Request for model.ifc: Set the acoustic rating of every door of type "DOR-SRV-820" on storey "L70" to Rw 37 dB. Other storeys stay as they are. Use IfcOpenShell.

First a look at what the model holds.

```python
import ifcopenshell
import ifcopenshell.util.element

model = ifcopenshell.open("model.ifc")
print(model.schema)
storey = next(s for s in model.by_type("IfcBuildingStorey") if s.Name == "L70")
doors = [e for e in ifcopenshell.util.element.get_decomposition(storey) if e.is_a("IfcDoor")]
seen = {}
for e in doors:
    element_type = ifcopenshell.util.element.get_type(e)
    key = (element_type.Name if element_type != e and element_type else None, ifcopenshell.util.element.get_pset(e, "Pset_DoorCommon", "AcousticRating"))
    seen[key] = seen.get(key, 0) + 1
for (name, value), count in sorted(seen.items(), key=str):
    print(count, "x", name, "|", value)
```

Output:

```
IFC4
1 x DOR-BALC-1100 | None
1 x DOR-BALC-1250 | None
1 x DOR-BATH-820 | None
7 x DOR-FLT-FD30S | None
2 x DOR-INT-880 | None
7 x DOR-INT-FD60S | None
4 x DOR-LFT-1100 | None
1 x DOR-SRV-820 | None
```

```python
import ifcopenshell
import ifcopenshell.api.pset
import ifcopenshell.util.element

model = ifcopenshell.open("model.ifc")

storey = next(s for s in model.by_type("IfcBuildingStorey") if s.Name == "L70")
doors = [e for e in ifcopenshell.util.element.get_decomposition(storey) if e.is_a("IfcDoor")]

count = 0
for e in doors:
    element_type = ifcopenshell.util.element.get_type(e)
    if element_type in (None, e) or element_type.Name != "DOR-SRV-820":
        continue
    found = ifcopenshell.util.element.get_pset(e, "Pset_DoorCommon", should_inherit=False)
    if found:
        pset = model.by_id(found["id"])
        if len(ifcopenshell.util.element.get_elements_by_pset(pset)) > 1:
            pset = ifcopenshell.api.pset.unshare_pset(model, products=[e], pset=pset)[0]
    else:
        pset = ifcopenshell.api.pset.add_pset(model, product=e, name="Pset_DoorCommon")
    ifcopenshell.api.pset.edit_pset(model, pset=pset, properties={"AcousticRating": "Rw 37 dB"})
    count += 1

print(count, "doors updated")

model.write("model_rev.ifc")
```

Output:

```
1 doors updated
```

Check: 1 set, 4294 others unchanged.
